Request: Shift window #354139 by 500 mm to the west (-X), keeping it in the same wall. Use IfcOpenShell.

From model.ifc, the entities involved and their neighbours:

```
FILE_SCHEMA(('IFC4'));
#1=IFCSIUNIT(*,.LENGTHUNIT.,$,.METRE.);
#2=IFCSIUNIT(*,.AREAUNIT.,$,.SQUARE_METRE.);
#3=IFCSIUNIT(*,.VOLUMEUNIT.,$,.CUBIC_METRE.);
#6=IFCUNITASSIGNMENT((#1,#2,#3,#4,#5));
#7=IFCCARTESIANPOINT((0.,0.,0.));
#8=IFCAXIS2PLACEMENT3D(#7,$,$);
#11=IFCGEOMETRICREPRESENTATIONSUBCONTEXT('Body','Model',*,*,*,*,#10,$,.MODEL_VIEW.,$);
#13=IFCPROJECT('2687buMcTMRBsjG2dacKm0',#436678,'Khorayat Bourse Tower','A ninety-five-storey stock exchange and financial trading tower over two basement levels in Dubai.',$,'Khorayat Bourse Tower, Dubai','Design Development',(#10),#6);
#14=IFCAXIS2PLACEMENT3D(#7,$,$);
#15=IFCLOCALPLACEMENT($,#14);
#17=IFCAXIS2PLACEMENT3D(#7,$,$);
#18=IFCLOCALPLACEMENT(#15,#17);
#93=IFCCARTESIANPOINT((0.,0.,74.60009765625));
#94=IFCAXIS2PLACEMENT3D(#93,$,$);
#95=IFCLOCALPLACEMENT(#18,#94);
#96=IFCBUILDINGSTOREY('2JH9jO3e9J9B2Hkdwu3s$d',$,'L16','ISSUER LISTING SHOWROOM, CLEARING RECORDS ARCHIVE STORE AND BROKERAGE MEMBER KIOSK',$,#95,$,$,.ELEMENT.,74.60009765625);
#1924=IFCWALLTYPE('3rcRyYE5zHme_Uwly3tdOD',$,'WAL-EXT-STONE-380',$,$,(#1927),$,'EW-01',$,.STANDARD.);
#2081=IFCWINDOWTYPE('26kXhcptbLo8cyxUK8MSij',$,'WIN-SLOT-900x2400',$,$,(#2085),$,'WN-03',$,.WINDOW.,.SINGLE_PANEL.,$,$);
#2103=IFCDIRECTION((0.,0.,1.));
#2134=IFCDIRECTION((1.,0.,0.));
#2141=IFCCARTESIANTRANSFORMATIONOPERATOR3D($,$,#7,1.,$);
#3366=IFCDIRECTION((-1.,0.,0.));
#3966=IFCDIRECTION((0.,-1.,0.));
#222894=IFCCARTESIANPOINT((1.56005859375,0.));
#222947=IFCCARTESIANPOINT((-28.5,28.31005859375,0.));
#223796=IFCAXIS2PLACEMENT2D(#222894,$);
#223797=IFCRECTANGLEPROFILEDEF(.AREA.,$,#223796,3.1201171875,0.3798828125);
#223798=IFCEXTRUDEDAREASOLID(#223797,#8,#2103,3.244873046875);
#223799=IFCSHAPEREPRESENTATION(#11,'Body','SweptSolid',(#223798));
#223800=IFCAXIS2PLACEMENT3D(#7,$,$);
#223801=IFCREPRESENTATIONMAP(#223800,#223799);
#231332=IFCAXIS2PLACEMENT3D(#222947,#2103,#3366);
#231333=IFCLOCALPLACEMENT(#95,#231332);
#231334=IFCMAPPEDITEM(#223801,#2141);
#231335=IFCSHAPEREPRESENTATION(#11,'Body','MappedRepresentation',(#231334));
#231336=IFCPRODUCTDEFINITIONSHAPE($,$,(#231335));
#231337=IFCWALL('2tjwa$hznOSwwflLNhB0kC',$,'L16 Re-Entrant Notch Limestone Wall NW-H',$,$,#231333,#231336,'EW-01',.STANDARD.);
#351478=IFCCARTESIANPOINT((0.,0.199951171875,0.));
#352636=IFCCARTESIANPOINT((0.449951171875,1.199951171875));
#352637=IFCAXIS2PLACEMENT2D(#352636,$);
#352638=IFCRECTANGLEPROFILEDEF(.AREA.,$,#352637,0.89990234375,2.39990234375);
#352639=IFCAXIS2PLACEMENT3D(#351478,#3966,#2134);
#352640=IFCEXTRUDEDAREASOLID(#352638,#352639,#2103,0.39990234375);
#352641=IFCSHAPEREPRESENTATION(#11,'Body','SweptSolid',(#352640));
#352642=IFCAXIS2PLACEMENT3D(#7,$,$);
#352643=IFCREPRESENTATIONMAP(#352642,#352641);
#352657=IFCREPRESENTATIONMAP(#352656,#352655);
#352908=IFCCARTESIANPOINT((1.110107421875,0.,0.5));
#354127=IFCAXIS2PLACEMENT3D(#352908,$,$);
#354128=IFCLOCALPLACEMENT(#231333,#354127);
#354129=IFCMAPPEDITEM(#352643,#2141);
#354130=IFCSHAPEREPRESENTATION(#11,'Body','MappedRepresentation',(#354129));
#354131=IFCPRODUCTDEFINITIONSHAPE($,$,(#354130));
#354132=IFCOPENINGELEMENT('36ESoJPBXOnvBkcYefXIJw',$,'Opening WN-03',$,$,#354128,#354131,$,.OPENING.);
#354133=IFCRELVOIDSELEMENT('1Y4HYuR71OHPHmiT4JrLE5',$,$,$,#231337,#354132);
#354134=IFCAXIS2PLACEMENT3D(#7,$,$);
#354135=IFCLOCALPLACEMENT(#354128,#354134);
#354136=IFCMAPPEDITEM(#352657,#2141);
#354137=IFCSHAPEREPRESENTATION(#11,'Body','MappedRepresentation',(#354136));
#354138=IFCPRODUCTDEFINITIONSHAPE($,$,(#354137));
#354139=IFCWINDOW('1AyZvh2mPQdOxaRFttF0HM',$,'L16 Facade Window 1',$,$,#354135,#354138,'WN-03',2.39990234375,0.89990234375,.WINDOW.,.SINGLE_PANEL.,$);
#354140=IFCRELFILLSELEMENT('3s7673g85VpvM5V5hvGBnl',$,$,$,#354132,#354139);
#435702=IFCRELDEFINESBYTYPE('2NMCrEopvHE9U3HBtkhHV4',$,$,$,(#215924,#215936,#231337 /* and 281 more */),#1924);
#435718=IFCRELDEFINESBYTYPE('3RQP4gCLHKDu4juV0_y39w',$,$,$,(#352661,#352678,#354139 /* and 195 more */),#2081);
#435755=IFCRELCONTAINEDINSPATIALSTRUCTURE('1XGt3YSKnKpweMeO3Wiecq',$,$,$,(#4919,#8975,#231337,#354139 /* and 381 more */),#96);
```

```python
import ifcopenshell
import ifcopenshell.api.geometry
import ifcopenshell.util.placement

model = ifcopenshell.open("model.ifc")

window = model.by_guid("1AyZvh2mPQdOxaRFttF0HM")
opening = window.FillsVoids[0].RelatingOpeningElement
wall = opening.VoidsElements[0].RelatingBuildingElement

wall_matrix = ifcopenshell.util.placement.get_local_placement(wall.ObjectPlacement)
shift = wall_matrix[:3, 0] * 0.5
before = ifcopenshell.util.placement.get_local_placement(window.ObjectPlacement)[:3, 3].copy()

# The window is placed relative to its opening, so it follows when the opening moves.
matrix = ifcopenshell.util.placement.get_local_placement(opening.ObjectPlacement)
matrix[:3, 3] += shift
ifcopenshell.api.geometry.edit_object_placement(
    model, product=opening, matrix=matrix, is_si=False, should_transform_children=True
)

after = ifcopenshell.util.placement.get_local_placement(window.ObjectPlacement)[:3, 3]
print("window moved by", (after - before).round(3) + 0.0)

model.write("model_v2.ifc")
```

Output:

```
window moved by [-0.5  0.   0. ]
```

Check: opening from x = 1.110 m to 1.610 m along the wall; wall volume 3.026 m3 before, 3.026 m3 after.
